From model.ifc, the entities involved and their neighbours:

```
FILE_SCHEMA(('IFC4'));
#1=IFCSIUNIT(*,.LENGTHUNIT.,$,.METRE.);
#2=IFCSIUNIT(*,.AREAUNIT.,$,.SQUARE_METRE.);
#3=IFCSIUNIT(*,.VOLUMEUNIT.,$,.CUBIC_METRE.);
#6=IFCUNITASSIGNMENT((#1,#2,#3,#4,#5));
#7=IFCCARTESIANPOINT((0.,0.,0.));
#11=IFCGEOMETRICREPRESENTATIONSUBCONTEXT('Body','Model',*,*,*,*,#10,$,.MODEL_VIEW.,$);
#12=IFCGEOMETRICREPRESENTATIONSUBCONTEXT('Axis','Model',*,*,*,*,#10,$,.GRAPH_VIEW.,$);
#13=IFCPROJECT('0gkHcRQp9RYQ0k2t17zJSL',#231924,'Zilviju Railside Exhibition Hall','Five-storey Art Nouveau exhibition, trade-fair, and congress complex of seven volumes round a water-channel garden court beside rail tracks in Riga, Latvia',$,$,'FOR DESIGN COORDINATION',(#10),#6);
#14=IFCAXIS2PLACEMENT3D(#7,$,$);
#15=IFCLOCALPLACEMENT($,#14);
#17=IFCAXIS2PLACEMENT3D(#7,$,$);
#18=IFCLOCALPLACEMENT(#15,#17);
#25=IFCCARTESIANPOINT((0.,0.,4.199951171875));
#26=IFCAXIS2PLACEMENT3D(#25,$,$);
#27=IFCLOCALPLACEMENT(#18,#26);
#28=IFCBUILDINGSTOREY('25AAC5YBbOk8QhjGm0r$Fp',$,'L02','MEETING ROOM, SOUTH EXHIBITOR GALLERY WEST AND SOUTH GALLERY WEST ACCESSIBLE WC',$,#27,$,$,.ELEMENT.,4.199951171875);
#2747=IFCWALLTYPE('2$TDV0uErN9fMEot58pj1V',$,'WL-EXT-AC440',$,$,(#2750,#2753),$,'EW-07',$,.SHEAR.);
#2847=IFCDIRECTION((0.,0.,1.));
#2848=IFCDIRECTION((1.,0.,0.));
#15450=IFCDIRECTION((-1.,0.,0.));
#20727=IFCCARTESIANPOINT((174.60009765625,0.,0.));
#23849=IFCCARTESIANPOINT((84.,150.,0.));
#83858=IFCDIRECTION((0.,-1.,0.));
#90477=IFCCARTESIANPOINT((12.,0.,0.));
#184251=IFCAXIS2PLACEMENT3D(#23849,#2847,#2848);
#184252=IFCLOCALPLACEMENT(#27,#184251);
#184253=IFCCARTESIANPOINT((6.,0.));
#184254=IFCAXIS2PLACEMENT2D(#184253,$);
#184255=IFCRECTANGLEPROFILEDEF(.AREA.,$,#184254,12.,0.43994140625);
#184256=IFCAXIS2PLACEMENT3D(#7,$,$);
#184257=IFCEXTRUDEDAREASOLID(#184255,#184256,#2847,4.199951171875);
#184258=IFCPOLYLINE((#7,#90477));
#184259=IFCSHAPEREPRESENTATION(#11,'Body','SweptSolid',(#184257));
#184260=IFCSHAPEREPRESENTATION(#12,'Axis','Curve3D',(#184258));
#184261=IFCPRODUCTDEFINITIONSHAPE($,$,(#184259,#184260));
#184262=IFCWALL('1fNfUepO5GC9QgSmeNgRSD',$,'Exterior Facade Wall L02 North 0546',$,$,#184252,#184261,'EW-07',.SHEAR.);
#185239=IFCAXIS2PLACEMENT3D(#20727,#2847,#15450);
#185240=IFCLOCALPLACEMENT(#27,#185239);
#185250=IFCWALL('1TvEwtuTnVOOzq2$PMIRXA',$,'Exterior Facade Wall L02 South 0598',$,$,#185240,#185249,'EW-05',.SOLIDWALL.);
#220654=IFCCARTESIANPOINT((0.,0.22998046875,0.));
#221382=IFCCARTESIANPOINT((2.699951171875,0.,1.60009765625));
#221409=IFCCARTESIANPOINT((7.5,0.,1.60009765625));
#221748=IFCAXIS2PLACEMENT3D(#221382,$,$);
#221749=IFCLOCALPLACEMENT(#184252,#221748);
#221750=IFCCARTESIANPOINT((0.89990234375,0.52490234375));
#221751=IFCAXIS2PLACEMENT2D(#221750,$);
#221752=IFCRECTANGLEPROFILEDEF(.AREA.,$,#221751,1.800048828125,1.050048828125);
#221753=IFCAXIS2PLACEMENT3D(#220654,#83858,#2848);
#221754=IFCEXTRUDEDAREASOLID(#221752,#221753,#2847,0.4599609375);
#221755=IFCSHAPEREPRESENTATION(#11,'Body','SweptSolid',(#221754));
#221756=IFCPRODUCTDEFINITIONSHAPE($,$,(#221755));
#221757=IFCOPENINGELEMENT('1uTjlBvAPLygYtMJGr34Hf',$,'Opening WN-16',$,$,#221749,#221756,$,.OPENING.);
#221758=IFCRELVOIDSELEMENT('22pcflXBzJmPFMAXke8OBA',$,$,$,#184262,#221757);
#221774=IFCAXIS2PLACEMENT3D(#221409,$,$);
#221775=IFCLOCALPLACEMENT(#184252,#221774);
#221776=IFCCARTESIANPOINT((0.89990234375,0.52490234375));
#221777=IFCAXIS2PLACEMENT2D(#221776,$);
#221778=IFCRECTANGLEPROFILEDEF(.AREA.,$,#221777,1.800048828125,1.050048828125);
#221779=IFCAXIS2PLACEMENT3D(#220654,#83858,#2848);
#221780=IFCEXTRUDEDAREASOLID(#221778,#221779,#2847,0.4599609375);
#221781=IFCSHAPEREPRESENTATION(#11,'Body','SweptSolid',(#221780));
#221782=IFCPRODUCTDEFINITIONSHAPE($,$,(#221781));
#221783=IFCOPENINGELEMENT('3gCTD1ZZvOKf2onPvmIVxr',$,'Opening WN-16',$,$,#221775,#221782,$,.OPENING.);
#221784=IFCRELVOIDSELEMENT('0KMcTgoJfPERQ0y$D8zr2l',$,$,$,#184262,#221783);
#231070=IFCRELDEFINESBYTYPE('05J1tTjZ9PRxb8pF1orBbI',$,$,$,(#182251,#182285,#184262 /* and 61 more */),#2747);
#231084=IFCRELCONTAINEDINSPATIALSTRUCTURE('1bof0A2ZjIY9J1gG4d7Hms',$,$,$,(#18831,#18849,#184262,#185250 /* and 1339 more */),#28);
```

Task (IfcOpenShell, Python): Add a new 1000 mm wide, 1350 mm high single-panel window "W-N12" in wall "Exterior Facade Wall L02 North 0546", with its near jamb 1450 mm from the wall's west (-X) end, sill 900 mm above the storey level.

```python
import numpy as np
import ifcopenshell
import ifcopenshell.api.feature
import ifcopenshell.api.geometry
import ifcopenshell.api.root
import ifcopenshell.api.spatial
import ifcopenshell.geom
import ifcopenshell.util.element
import ifcopenshell.util.placement
import ifcopenshell.util.representation
import ifcopenshell.util.shape
import ifcopenshell.util.unit

model = ifcopenshell.open("model.ifc")
unit_scale = ifcopenshell.util.unit.calculate_unit_scale(model)
settings = ifcopenshell.geom.settings()


def volume(element):
    """Net volume in cubic metres, openings subtracted."""
    shape = ifcopenshell.geom.create_shape(settings, element)
    return ifcopenshell.util.shape.get_volume(shape.geometry)


wall = model.by_id(184262)
storey = ifcopenshell.util.element.get_container(wall, ifc_class="IfcBuildingStorey")
context = ifcopenshell.util.representation.get_context(model, "Model", "Body", "MODEL_VIEW")
before = volume(wall)

width, height, from_end, sill = 1, 1.35, 1.45, 0.9  # metres

# The wall runs along its own X axis, and the end named is its -X end.
wall_shape = ifcopenshell.geom.create_shape(settings, wall)
x, y, z = ifcopenshell.util.shape.get_vertices(wall_shape.geometry).T
start = x.min() + from_end
face, thickness = float(y.min()), float(y.max() - y.min())
wall_matrix = ifcopenshell.util.placement.get_local_placement(wall.ObjectPlacement)
level = ifcopenshell.util.placement.get_local_placement(storey.ObjectPlacement)[2, 3]


def in_wall(x, y):
    """Placement at x, y metres in the wall's axes, at sill height."""
    matrix = wall_matrix.copy()
    matrix[:, 3] = wall_matrix @ np.array([x / unit_scale, y / unit_scale, 0.0, 1.0])
    matrix[2, 3] = level + sill / unit_scale
    return matrix


# Opening: a box that overshoots both wall faces by 50 mm.
opening = ifcopenshell.api.root.create_entity(model, ifc_class="IfcOpeningElement", predefined_type="OPENING")
box = ifcopenshell.api.geometry.add_wall_representation(
    model, context=context, length=width, height=height, thickness=thickness + 0.1
)
ifcopenshell.api.geometry.assign_representation(model, product=opening, representation=box)
ifcopenshell.api.geometry.edit_object_placement(model, product=opening, matrix=in_wall(start, face - 0.05), is_si=False)
ifcopenshell.api.feature.add_feature(model, feature=opening, element=wall)

window = ifcopenshell.api.root.create_entity(model, ifc_class="IfcWindow", name="W-N12", predefined_type="WINDOW")
window.OverallWidth, window.OverallHeight = width / unit_scale, height / unit_scale
window.PartitioningType = "SINGLE_PANEL"
body = ifcopenshell.api.geometry.add_window_representation(
    model,
    context=context,
    overall_width=window.OverallWidth,
    overall_height=window.OverallHeight,
    partition_type="SINGLE_PANEL",
)
ifcopenshell.api.geometry.assign_representation(model, product=window, representation=body)
ifcopenshell.api.spatial.assign_container(model, products=[window], relating_structure=storey)
ifcopenshell.api.feature.add_filling(model, opening=opening, element=window)

# Centre the window in the wall's thickness.
ifcopenshell.api.geometry.edit_object_placement(model, product=window, matrix=in_wall(start, face), is_si=False)
window_shape = ifcopenshell.geom.create_shape(settings, window)
depth = ifcopenshell.util.shape.get_vertices(window_shape.geometry)[:, 1]
offset = face + thickness / 2 - (depth.min() + depth.max()) / 2
ifcopenshell.api.geometry.edit_object_placement(model, product=window, matrix=in_wall(start, offset), is_si=False)

after = volume(wall)

print(f"wall volume {before:.3f} -> {after:.3f} m3")

model.write("model_rev.ifc")
```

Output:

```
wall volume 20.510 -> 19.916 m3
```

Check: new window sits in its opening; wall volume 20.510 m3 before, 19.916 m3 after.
